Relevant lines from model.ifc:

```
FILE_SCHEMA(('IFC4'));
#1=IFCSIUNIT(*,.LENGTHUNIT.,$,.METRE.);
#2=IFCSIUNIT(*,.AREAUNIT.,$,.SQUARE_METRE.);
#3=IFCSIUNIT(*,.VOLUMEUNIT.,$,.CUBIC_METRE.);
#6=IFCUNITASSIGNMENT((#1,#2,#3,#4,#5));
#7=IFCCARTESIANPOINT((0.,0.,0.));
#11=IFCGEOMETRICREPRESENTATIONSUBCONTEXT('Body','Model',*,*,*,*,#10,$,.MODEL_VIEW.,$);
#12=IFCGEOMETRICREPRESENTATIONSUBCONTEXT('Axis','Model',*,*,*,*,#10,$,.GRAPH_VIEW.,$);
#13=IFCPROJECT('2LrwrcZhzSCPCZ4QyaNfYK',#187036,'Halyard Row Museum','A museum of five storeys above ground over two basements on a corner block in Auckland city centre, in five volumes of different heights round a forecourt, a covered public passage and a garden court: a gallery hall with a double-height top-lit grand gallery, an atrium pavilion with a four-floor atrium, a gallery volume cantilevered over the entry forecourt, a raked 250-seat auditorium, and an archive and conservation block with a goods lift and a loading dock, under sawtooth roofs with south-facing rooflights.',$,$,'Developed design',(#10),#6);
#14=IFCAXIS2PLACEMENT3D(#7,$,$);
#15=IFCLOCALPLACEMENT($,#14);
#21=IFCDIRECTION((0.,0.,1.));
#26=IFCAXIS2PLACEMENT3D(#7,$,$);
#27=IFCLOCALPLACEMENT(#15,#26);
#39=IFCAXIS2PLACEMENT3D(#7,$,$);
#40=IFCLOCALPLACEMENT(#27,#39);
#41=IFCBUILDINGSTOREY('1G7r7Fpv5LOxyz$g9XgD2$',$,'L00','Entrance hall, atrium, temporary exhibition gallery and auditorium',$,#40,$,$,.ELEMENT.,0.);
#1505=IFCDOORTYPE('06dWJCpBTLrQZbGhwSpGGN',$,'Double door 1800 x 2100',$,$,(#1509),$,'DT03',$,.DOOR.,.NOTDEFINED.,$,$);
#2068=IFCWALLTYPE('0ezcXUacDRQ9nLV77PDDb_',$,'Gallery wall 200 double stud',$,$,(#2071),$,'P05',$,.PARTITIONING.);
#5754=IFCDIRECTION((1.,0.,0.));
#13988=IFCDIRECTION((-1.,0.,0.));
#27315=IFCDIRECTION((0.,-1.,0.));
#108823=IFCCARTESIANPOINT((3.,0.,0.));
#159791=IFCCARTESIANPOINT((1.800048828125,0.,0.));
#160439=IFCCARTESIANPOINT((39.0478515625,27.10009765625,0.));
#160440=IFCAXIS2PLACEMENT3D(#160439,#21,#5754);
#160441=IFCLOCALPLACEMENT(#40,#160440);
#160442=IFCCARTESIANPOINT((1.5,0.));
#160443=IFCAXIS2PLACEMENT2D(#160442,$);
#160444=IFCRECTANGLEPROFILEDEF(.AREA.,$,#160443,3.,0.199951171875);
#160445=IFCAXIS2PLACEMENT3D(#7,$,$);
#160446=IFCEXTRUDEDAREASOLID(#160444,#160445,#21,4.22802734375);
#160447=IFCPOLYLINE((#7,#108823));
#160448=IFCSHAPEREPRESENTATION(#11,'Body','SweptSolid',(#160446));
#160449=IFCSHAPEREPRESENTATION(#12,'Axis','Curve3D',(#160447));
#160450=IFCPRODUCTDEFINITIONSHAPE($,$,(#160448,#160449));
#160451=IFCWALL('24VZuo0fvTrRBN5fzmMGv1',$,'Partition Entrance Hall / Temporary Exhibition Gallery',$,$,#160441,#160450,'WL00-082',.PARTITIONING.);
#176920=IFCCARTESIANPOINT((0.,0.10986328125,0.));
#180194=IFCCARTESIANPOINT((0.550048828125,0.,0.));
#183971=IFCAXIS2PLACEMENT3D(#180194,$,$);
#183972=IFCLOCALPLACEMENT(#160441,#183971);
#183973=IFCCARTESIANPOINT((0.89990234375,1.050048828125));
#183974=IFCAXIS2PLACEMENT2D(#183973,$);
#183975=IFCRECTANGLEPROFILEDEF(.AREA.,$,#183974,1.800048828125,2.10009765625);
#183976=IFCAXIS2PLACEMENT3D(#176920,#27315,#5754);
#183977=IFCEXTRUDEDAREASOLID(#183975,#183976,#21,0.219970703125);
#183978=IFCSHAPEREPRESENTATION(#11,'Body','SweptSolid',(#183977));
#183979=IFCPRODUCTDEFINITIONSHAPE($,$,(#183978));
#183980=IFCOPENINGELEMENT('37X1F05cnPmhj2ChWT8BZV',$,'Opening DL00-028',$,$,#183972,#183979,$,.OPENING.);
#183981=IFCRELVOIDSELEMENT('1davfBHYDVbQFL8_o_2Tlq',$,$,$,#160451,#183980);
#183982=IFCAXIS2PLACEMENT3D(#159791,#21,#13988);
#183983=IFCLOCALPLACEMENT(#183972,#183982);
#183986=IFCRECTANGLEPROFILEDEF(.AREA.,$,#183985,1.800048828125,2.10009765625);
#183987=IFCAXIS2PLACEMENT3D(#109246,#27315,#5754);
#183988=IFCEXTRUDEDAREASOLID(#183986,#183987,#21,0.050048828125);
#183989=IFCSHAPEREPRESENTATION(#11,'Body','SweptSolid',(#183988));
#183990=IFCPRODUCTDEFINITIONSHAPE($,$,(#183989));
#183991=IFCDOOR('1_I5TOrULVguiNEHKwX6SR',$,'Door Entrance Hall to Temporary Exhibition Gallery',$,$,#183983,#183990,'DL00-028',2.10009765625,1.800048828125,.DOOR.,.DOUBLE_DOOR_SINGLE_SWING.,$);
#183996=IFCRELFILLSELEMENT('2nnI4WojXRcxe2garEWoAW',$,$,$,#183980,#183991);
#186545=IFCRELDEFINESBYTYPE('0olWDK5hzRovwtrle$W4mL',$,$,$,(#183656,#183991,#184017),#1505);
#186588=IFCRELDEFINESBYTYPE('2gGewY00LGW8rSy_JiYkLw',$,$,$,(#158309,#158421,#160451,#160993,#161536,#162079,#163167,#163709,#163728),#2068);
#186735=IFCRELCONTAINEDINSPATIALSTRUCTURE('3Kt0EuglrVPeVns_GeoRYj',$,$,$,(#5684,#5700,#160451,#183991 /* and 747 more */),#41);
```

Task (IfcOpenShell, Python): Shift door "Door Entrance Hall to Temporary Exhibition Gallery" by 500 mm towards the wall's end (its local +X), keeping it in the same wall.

```python
import ifcopenshell
import ifcopenshell.api.geometry
import ifcopenshell.util.placement
import ifcopenshell.util.unit

model = ifcopenshell.open("model.ifc")
unit_scale = ifcopenshell.util.unit.calculate_unit_scale(model)

door = model.by_guid("1_I5TOrULVguiNEHKwX6SR")
opening = door.FillsVoids[0].RelatingOpeningElement
wall = opening.VoidsElements[0].RelatingBuildingElement

wall_matrix = ifcopenshell.util.placement.get_local_placement(wall.ObjectPlacement)
shift = wall_matrix[:3, 0] * 0.5 / unit_scale
before = ifcopenshell.util.placement.get_local_placement(door.ObjectPlacement)[:3, 3].copy()

# The door is placed relative to its opening, so it follows when the opening moves.
matrix = ifcopenshell.util.placement.get_local_placement(opening.ObjectPlacement)
matrix[:3, 3] += shift
ifcopenshell.api.geometry.edit_object_placement(
    model, product=opening, matrix=matrix, is_si=False, should_transform_children=True
)

after = ifcopenshell.util.placement.get_local_placement(door.ObjectPlacement)[:3, 3]
print("door moved by", (after - before).round(3) + 0.0)

model.write("model_edited.ifc")
```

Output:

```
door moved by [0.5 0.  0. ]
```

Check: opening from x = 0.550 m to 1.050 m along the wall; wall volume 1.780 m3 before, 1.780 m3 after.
